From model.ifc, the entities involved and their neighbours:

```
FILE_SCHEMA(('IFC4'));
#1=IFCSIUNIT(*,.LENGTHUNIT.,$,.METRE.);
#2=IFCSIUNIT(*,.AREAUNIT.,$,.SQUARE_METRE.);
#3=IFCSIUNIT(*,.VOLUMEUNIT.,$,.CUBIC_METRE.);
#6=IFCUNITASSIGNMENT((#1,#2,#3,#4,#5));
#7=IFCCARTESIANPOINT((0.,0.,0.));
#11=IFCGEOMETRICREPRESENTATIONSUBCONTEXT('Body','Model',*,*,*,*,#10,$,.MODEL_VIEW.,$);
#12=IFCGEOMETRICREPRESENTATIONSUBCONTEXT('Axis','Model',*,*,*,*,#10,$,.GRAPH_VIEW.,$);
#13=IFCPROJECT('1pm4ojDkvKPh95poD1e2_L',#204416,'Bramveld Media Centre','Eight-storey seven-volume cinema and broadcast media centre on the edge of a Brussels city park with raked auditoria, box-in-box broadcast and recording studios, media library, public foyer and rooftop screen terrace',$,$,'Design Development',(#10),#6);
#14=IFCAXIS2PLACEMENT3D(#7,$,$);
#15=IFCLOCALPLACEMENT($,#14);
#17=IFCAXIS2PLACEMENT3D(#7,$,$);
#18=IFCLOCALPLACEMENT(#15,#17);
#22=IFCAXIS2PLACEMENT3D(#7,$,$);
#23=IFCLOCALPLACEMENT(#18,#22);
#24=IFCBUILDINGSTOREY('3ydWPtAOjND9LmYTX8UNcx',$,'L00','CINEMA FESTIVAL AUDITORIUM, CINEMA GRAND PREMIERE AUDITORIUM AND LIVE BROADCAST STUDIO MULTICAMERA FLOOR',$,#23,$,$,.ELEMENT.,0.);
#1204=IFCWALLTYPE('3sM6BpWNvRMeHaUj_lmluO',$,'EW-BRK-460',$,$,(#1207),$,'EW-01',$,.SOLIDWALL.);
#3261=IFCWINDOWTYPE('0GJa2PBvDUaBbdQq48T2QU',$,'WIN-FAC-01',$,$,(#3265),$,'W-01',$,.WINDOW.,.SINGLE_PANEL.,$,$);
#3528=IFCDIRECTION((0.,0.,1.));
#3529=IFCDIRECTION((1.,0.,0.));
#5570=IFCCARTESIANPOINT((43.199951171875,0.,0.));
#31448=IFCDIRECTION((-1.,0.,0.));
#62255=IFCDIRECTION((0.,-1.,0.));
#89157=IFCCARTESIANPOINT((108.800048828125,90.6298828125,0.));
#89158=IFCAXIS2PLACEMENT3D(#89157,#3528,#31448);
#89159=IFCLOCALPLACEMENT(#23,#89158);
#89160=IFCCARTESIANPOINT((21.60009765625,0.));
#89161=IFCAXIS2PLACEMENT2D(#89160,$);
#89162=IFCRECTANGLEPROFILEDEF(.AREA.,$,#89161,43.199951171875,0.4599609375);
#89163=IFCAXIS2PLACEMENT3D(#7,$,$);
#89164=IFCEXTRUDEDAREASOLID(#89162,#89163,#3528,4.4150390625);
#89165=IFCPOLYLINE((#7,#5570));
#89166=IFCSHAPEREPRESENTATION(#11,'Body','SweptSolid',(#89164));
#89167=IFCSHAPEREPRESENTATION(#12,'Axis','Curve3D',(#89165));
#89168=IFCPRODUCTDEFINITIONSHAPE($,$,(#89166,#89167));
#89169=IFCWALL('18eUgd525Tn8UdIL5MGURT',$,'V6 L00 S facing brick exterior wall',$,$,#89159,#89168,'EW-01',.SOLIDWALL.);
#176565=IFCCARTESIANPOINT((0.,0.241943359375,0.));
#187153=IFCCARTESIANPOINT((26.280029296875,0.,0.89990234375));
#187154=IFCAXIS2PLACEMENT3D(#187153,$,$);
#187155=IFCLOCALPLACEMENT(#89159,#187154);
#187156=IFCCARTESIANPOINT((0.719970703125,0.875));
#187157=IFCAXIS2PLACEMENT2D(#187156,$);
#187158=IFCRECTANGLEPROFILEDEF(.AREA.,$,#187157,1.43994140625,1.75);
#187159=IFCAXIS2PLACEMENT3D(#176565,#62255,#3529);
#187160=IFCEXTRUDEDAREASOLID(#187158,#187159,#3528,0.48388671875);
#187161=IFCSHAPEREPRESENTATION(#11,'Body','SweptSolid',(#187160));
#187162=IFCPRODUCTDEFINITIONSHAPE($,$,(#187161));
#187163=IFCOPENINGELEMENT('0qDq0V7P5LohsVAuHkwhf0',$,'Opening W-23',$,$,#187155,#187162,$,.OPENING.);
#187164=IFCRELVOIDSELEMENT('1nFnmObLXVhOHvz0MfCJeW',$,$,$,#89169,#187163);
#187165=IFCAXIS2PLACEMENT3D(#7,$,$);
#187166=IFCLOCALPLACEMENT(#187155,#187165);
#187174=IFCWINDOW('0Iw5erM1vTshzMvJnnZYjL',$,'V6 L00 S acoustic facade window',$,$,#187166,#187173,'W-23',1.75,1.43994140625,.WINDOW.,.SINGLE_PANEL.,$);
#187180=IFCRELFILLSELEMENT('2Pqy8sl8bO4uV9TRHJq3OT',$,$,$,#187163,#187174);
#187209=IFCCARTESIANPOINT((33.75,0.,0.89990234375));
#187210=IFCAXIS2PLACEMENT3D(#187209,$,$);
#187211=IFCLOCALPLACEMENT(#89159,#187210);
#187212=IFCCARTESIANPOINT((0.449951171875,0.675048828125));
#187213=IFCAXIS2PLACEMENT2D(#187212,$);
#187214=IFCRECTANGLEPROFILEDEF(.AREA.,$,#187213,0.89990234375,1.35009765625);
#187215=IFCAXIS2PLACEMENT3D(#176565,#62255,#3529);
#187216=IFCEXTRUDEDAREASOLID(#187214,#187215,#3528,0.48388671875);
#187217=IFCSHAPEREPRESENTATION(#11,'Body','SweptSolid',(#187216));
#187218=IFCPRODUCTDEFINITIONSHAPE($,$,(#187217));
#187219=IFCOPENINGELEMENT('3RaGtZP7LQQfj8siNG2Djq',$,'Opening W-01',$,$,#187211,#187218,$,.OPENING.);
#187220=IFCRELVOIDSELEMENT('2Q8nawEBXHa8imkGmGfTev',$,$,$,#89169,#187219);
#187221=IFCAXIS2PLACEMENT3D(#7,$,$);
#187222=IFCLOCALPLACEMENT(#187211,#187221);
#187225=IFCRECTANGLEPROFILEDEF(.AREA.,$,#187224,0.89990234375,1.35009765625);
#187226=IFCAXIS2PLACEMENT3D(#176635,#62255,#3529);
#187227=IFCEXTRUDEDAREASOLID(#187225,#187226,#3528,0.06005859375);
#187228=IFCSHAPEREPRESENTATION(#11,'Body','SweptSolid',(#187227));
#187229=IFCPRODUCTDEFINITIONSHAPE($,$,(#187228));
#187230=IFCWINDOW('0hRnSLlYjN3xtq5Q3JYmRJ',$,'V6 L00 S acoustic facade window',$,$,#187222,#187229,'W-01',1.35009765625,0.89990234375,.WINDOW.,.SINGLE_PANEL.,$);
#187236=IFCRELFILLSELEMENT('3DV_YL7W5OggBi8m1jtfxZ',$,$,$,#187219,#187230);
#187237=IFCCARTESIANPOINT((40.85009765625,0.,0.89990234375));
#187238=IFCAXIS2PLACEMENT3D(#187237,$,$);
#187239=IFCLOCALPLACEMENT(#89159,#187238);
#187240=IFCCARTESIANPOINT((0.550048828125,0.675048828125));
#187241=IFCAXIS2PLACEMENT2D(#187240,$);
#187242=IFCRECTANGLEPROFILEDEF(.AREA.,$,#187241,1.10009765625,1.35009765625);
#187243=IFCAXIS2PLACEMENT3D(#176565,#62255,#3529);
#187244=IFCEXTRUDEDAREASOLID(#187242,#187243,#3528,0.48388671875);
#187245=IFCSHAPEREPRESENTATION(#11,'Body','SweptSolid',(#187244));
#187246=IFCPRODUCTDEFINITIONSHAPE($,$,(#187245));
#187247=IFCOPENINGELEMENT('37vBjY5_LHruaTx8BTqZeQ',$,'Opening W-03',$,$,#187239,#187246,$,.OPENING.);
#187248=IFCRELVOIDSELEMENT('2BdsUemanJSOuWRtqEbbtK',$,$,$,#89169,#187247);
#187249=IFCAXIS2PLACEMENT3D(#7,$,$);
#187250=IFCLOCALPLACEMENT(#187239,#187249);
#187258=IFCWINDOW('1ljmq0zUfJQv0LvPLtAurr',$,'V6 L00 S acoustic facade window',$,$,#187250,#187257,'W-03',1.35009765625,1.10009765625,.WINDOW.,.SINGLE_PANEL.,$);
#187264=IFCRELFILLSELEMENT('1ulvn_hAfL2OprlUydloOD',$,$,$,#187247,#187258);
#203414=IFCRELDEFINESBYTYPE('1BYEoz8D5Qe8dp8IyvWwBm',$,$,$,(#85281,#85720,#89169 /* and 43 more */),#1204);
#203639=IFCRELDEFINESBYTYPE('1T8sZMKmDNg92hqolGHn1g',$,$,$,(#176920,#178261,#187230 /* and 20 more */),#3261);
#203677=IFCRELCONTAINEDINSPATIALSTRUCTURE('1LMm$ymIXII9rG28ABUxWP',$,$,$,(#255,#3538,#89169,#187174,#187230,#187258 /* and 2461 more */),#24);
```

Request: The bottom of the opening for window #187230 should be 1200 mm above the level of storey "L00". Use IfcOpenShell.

```python
import numpy as np
import ifcopenshell
import ifcopenshell.api.geometry
import ifcopenshell.geom
import ifcopenshell.util.element
import ifcopenshell.util.placement
import ifcopenshell.util.shape
import ifcopenshell.util.unit

model = ifcopenshell.open("model.ifc")
unit_scale = ifcopenshell.util.unit.calculate_unit_scale(model)

window = model.by_guid("0hRnSLlYjN3xtq5Q3JYmRJ")
opening = window.FillsVoids[0].RelatingOpeningElement
storey = ifcopenshell.util.element.get_container(window, ifc_class="IfcBuildingStorey")
level = ifcopenshell.util.placement.get_local_placement(storey.ObjectPlacement)[2, 3]

# The opening's origin need not be at the sill, so measure its lowest point.
shape = ifcopenshell.geom.create_shape(ifcopenshell.geom.settings(), opening)
bottom = ifcopenshell.util.shape.get_shape_bottom_elevation(shape, shape.geometry) / unit_scale
dz = level + 1.2 / unit_scale - bottom

shift = np.array([0.0, 0.0, dz])
# The window is placed relative to its opening, so it follows when the opening moves.
matrix = ifcopenshell.util.placement.get_local_placement(opening.ObjectPlacement)
matrix[:3, 3] += shift
ifcopenshell.api.geometry.edit_object_placement(
    model, product=opening, matrix=matrix, is_si=False, should_transform_children=True
)

print(f"moved by {dz * unit_scale:+.3f} m")

model.write("model_edited.ifc")
```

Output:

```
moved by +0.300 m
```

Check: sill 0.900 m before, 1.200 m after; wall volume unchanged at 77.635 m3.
